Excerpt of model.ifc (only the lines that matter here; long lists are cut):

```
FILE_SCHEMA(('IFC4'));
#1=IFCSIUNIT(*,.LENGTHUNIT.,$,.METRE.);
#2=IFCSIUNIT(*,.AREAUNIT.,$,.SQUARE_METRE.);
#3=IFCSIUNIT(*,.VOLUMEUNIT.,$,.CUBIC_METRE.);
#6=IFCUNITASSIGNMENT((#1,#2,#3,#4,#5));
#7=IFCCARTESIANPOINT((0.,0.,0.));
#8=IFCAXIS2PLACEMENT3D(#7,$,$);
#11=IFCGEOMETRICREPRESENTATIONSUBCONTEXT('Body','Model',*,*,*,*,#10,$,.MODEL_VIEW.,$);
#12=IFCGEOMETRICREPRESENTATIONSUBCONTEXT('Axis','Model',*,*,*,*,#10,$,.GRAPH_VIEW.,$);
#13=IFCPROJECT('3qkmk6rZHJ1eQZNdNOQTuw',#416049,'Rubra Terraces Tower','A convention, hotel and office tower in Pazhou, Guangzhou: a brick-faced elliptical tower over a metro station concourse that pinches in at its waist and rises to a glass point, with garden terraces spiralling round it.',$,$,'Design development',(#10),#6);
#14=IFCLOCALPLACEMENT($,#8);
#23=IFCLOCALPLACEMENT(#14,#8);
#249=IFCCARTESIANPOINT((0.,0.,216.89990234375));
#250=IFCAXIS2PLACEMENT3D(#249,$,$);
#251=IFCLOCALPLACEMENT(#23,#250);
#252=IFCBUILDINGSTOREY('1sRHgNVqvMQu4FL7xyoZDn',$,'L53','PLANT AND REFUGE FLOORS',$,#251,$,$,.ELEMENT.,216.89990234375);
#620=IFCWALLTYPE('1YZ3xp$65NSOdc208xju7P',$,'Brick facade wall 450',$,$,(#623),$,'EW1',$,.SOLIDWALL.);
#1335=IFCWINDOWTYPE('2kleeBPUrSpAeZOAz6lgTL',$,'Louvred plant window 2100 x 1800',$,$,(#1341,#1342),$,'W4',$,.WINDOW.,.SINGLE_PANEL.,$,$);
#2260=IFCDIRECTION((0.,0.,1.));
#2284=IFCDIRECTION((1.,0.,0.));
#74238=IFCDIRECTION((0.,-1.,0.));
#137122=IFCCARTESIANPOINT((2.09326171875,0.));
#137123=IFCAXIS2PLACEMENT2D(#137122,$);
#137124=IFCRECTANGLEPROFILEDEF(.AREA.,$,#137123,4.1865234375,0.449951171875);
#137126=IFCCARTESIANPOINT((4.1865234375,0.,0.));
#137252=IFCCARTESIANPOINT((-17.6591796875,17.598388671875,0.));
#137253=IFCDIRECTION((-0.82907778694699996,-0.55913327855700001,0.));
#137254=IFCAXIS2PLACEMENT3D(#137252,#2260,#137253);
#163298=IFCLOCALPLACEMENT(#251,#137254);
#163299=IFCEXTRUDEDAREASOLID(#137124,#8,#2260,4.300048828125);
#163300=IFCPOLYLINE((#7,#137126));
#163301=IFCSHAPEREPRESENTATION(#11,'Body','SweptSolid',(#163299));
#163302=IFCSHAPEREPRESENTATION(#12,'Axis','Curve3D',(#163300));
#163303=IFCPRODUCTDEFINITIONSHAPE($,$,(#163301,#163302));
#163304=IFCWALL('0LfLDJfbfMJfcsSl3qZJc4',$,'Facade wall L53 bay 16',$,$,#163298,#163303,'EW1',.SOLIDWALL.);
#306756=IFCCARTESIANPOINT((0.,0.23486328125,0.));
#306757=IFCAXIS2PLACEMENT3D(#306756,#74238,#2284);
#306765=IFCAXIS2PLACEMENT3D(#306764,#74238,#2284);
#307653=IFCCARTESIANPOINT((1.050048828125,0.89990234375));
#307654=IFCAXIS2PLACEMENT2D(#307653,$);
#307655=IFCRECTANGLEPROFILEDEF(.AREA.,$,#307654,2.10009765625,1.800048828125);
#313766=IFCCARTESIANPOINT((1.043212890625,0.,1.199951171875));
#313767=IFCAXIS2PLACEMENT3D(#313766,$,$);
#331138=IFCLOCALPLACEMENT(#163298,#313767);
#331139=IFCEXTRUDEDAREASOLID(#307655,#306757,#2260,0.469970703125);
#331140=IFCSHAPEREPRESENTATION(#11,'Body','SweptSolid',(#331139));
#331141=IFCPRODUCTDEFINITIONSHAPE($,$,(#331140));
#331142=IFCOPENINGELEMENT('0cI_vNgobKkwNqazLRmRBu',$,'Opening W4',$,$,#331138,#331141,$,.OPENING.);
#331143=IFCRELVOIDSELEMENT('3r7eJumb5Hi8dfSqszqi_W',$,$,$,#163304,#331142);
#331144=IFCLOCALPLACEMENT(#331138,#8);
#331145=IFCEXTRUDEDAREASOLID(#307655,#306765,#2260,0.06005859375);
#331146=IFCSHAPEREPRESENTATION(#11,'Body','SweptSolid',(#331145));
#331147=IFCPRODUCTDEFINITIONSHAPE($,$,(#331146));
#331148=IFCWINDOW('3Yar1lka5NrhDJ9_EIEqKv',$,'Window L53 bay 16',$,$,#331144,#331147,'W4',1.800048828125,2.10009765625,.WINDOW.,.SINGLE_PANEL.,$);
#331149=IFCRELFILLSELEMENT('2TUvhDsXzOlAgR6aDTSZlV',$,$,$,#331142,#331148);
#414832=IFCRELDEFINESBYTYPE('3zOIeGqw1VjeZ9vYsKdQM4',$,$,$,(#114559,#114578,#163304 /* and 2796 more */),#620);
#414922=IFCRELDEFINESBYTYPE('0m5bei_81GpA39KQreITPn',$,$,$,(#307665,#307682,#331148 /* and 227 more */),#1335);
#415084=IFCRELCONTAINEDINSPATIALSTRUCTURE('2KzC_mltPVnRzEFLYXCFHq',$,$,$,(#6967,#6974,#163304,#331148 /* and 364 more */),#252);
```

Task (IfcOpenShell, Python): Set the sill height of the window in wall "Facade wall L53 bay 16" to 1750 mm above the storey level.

```python
import numpy as np
import ifcopenshell
import ifcopenshell.api.geometry
import ifcopenshell.geom
import ifcopenshell.util.element
import ifcopenshell.util.placement
import ifcopenshell.util.shape
import ifcopenshell.util.unit

model = ifcopenshell.open("model.ifc")
unit_scale = ifcopenshell.util.unit.calculate_unit_scale(model)

window = model.by_guid("3Yar1lka5NrhDJ9_EIEqKv")
opening = window.FillsVoids[0].RelatingOpeningElement
storey = ifcopenshell.util.element.get_container(window, ifc_class="IfcBuildingStorey")
level = ifcopenshell.util.placement.get_local_placement(storey.ObjectPlacement)[2, 3]

# The opening's origin need not be at the sill, so measure its lowest point.
shape = ifcopenshell.geom.create_shape(ifcopenshell.geom.settings(), opening)
bottom = ifcopenshell.util.shape.get_shape_bottom_elevation(shape, shape.geometry) / unit_scale
dz = level + 1.75 / unit_scale - bottom

shift = np.array([0.0, 0.0, dz])
# The window is placed relative to its opening, so it follows when the opening moves.
matrix = ifcopenshell.util.placement.get_local_placement(opening.ObjectPlacement)
matrix[:3, 3] += shift
ifcopenshell.api.geometry.edit_object_placement(
    model, product=opening, matrix=matrix, is_si=False, should_transform_children=True
)

print(f"moved by {dz * unit_scale:+.3f} m")

model.write("model_v2.ifc")
```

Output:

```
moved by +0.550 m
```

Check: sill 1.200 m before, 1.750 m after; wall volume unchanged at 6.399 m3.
